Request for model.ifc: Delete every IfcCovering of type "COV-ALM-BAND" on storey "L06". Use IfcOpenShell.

First a look at what the model holds.

```python
import ifcopenshell
import ifcopenshell.util.element

model = ifcopenshell.open("model.ifc")
print(model.schema)
storey = next(s for s in model.by_type("IfcBuildingStorey") if s.Name == "L06")
coverings = [e for e in ifcopenshell.util.element.get_decomposition(storey) if e.is_a("IfcCovering")]
seen = {}
for e in coverings:
    element_type = ifcopenshell.util.element.get_type(e)
    name = element_type.Name if element_type not in (None, e) else None
    seen[name] = seen.get(name, 0) + 1
for name, count in sorted(seen.items(), key=str):
    print(count, "x", name)
```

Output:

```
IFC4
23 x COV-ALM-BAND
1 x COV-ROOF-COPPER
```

```python
import ifcopenshell
import ifcopenshell.api.root
import ifcopenshell.util.element

model = ifcopenshell.open("model.ifc")

storey = next(s for s in model.by_type("IfcBuildingStorey") if s.Name == "L06")
coverings = [e for e in ifcopenshell.util.element.get_decomposition(storey) if e.is_a("IfcCovering")]
targets = [e for e in coverings if (t := ifcopenshell.util.element.get_type(e)) not in (None, e) and t.Name == "COV-ALM-BAND"]

for e in targets:
    ifcopenshell.api.root.remove_product(model, product=e)
print(len(targets), "removed")

model.write("model_rev.ifc")
```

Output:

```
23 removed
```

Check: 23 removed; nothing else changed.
